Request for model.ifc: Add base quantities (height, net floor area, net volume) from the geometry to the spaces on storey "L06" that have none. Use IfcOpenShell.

First a look at what the model holds.

```python
import ifcopenshell
import ifcopenshell.util.element
import ifcopenshell.util.unit

model = ifcopenshell.open("model.ifc")
print(model.schema)
for unit_type in ("LENGTHUNIT", "AREAUNIT", "VOLUMEUNIT"):
    print(unit_type, ifcopenshell.util.unit.calculate_unit_scale(model, unit_type))
storey = next(s for s in model.by_type("IfcBuildingStorey") if s.Name == "L06")
spaces = [e for e in ifcopenshell.util.element.get_decomposition(storey) if e.is_a("IfcSpace")]
for e in sorted(spaces, key=lambda e: e.id()):
    print(e.id(), e.is_a(), e.Name, list(ifcopenshell.util.element.get_psets(e, qtos_only=True)), sep=" | ")
```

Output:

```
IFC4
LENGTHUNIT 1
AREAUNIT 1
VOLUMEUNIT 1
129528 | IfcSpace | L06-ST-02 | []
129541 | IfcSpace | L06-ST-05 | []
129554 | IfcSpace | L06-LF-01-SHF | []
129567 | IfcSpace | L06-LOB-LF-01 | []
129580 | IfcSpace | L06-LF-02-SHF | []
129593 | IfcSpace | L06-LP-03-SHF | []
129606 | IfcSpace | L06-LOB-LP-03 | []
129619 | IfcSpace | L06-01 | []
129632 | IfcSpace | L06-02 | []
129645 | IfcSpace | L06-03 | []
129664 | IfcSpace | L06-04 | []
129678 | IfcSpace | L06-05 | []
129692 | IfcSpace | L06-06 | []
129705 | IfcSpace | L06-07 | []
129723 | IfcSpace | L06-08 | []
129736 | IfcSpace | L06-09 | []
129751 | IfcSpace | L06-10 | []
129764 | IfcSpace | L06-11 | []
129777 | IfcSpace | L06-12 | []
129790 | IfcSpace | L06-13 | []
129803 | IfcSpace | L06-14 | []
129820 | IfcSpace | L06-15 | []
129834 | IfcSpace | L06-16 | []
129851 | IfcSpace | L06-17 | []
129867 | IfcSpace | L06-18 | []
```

```python
import ifcopenshell
import ifcopenshell.api.pset
import ifcopenshell.geom
import ifcopenshell.util.element
import ifcopenshell.util.shape
import ifcopenshell.util.unit

model = ifcopenshell.open("model.ifc")
unit_scale = ifcopenshell.util.unit.calculate_unit_scale(model)
area_scale = ifcopenshell.util.unit.calculate_unit_scale(model, "AREAUNIT")
volume_scale = ifcopenshell.util.unit.calculate_unit_scale(model, "VOLUMEUNIT")
settings = ifcopenshell.geom.settings()

storey = next(s for s in model.by_type("IfcBuildingStorey") if s.Name == "L06")
spaces = [e for e in ifcopenshell.util.element.get_decomposition(storey) if e.is_a("IfcSpace")]

for e in sorted(spaces, key=lambda e: e.id()):
    if ifcopenshell.util.element.get_psets(e, qtos_only=True, should_inherit=False):
        continue
    # Geometry comes back in metres, in the element's own axes.
    shape = ifcopenshell.geom.create_shape(settings, e)
    values = {
        "Height": ifcopenshell.util.shape.get_z(shape.geometry) / unit_scale,
        "NetFloorArea": ifcopenshell.util.shape.get_footprint_area(shape.geometry) / area_scale,
        "NetVolume": ifcopenshell.util.shape.get_volume(shape.geometry) / volume_scale,
    }
    qto = ifcopenshell.api.pset.add_qto(model, product=e, name="Qto_SpaceBaseQuantities")
    ifcopenshell.api.pset.edit_qto(model, qto=qto, properties=values)
    print(e.id(), {k: round(v, 3) for k, v in values.items()})

model.write("model-out.ifc")
```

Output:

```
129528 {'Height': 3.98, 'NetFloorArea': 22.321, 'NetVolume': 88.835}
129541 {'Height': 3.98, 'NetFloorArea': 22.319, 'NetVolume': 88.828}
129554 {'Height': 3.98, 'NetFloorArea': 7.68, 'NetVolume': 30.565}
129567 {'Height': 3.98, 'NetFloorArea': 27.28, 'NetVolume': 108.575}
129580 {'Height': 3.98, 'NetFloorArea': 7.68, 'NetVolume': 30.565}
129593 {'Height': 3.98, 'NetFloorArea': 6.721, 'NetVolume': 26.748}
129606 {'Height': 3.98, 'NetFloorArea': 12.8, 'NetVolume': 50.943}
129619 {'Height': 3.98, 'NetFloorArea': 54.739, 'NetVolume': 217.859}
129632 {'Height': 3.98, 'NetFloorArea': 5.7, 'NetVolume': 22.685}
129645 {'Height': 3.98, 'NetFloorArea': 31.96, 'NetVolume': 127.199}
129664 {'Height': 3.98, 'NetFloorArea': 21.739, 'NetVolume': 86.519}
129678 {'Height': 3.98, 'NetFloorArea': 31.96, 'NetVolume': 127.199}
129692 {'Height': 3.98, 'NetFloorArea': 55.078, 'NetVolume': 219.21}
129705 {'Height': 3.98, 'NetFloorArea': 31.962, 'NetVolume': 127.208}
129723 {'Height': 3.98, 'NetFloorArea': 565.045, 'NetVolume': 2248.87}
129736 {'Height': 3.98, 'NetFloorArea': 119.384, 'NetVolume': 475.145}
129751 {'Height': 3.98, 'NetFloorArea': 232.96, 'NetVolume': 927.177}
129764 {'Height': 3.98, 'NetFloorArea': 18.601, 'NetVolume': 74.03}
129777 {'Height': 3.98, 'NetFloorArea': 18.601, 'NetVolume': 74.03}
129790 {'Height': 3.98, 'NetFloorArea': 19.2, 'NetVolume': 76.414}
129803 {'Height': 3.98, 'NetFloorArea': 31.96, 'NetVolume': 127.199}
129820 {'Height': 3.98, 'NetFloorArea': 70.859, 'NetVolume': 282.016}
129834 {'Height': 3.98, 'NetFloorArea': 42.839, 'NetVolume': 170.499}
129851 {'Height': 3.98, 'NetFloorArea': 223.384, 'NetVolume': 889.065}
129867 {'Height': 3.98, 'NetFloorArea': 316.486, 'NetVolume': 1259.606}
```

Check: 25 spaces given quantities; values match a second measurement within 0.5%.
